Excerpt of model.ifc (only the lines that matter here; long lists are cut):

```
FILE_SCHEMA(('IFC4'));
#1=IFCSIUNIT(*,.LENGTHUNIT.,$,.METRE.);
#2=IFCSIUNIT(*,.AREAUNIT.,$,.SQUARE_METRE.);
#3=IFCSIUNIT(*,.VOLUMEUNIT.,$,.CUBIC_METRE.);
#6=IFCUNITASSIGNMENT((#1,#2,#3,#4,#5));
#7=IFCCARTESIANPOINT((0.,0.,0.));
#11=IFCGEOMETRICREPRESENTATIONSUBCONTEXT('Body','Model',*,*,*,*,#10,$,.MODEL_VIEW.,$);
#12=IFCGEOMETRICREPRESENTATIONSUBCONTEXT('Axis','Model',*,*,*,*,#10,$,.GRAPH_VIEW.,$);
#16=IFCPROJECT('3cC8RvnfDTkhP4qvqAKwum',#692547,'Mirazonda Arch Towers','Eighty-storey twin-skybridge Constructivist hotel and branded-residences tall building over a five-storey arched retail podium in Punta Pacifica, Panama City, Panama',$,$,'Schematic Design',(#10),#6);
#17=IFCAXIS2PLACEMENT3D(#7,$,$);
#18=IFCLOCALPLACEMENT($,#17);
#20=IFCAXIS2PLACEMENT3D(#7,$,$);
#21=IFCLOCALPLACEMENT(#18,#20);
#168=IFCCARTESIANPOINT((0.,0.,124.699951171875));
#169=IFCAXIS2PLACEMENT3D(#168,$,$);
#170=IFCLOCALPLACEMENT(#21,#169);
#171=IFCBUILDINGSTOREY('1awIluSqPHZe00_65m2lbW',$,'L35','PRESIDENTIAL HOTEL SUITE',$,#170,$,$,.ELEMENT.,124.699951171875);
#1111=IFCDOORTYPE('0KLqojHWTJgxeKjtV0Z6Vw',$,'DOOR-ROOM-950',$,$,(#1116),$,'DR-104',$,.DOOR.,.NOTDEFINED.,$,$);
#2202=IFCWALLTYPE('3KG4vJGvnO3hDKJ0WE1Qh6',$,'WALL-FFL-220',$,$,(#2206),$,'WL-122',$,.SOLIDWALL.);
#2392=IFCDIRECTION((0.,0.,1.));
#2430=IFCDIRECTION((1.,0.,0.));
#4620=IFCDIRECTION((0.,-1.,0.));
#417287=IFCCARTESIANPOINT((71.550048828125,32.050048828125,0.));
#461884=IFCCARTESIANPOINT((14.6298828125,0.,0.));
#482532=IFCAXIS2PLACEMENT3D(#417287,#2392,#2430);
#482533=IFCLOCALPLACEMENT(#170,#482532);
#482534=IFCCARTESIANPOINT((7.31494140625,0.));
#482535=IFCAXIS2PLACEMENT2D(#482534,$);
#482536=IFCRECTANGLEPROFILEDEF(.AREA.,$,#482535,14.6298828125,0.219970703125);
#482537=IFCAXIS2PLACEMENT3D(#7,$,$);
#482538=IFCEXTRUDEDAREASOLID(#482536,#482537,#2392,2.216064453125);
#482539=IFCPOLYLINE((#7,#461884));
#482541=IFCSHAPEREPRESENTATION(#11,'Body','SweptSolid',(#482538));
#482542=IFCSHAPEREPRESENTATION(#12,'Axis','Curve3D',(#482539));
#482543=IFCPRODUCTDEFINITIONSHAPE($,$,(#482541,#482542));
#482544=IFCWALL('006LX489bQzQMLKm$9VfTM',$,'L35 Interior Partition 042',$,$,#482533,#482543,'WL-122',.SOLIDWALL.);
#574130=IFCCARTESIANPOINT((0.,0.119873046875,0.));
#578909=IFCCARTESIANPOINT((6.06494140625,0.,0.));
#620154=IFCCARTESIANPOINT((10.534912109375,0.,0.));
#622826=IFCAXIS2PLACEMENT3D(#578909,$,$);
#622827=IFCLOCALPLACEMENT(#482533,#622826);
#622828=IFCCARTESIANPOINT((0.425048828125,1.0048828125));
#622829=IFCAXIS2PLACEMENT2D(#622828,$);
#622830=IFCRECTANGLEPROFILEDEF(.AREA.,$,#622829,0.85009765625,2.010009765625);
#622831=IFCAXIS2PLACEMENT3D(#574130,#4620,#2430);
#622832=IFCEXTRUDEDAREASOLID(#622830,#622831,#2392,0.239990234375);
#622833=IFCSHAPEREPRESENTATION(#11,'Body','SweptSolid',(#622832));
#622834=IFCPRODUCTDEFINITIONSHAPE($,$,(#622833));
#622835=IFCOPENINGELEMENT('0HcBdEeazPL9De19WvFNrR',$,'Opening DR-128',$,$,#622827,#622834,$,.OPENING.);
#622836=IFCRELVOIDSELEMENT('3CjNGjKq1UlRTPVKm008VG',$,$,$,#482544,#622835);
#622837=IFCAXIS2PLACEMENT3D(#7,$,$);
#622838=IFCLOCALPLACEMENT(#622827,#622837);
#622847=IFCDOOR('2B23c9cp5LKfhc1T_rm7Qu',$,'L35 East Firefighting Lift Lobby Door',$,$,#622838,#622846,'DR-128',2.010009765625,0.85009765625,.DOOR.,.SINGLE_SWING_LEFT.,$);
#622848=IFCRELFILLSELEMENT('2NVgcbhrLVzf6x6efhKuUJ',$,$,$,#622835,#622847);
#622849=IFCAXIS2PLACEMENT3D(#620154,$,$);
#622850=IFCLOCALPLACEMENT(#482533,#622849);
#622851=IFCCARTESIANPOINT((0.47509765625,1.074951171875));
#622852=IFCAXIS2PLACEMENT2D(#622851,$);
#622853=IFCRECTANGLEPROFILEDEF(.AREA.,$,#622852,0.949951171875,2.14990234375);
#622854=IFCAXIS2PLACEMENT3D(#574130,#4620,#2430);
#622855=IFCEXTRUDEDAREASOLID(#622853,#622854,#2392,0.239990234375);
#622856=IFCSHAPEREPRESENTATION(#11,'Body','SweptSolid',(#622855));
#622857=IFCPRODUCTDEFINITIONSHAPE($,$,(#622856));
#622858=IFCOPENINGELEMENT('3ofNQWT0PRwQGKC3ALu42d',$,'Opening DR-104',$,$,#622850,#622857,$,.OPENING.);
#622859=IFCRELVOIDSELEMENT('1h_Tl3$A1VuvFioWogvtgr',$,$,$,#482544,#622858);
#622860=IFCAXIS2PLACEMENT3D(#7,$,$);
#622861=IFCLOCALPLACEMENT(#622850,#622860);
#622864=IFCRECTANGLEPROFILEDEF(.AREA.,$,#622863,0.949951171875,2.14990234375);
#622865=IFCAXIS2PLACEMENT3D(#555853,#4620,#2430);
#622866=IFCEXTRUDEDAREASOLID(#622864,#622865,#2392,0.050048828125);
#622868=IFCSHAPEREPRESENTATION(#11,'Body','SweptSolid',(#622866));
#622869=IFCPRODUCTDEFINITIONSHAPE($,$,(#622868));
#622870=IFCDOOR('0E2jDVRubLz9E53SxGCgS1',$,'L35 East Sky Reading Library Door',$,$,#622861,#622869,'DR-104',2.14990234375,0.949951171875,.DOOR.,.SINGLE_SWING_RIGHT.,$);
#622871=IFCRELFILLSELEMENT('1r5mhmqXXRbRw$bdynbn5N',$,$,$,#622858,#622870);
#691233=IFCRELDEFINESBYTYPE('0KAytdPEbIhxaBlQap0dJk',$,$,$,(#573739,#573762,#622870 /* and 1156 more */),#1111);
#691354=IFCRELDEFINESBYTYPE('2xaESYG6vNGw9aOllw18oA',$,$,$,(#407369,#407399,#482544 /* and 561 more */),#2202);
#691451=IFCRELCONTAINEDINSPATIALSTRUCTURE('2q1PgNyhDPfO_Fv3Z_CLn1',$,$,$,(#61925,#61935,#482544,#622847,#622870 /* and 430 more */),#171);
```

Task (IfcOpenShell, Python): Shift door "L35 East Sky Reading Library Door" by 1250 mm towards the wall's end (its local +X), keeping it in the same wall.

```python
import ifcopenshell
import ifcopenshell.api.geometry
import ifcopenshell.util.placement

model = ifcopenshell.open("model.ifc")

door = model.by_id(622870)
opening = door.FillsVoids[0].RelatingOpeningElement
wall = opening.VoidsElements[0].RelatingBuildingElement

wall_matrix = ifcopenshell.util.placement.get_local_placement(wall.ObjectPlacement)
shift = wall_matrix[:3, 0] * 1.25
before = ifcopenshell.util.placement.get_local_placement(door.ObjectPlacement)[:3, 3].copy()

# The door is placed relative to its opening, so it follows when the opening moves.
matrix = ifcopenshell.util.placement.get_local_placement(opening.ObjectPlacement)
matrix[:3, 3] += shift
ifcopenshell.api.geometry.edit_object_placement(
    model, product=opening, matrix=matrix, is_si=False, should_transform_children=True
)

after = ifcopenshell.util.placement.get_local_placement(door.ObjectPlacement)[:3, 3]
print("door moved by", (after - before).round(3) + 0.0)

model.write("model_edited.ifc")
```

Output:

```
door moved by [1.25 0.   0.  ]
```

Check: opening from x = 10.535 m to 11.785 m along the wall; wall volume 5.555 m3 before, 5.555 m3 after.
